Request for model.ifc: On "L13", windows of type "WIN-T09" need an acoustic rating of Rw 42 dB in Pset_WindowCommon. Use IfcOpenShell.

First a look at what the model holds.

```python
import ifcopenshell
import ifcopenshell.util.element

model = ifcopenshell.open("model.ifc")
print(model.schema)
storey = next(s for s in model.by_type("IfcBuildingStorey") if s.Name == "L13")
windows = [e for e in ifcopenshell.util.element.get_decomposition(storey) if e.is_a("IfcWindow")]
seen = {}
for e in windows:
    element_type = ifcopenshell.util.element.get_type(e)
    key = (element_type.Name if element_type != e and element_type else None, ifcopenshell.util.element.get_pset(e, "Pset_WindowCommon", "AcousticRating"))
    seen[key] = seen.get(key, 0) + 1
for (name, value), count in sorted(seen.items(), key=str):
    print(count, "x", name, "|", value)
```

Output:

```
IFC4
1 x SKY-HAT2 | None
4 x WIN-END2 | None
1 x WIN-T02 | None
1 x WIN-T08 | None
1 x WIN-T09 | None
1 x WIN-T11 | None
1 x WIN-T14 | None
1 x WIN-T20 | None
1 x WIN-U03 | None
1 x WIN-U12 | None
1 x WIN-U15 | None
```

```python
import ifcopenshell
import ifcopenshell.api.pset
import ifcopenshell.util.element

model = ifcopenshell.open("model.ifc")

storey = next(s for s in model.by_type("IfcBuildingStorey") if s.Name == "L13")
windows = [e for e in ifcopenshell.util.element.get_decomposition(storey) if e.is_a("IfcWindow")]

count = 0
for e in windows:
    element_type = ifcopenshell.util.element.get_type(e)
    if element_type in (None, e) or element_type.Name != "WIN-T09":
        continue
    # add_pset returns the element's existing set when there is one.
    pset = ifcopenshell.api.pset.add_pset(model, product=e, name="Pset_WindowCommon")
    ifcopenshell.api.pset.edit_pset(model, pset=pset, properties={"AcousticRating": "Rw 42 dB"})
    count += 1

print(count, "windows updated")

model.write("model_updated.ifc")
```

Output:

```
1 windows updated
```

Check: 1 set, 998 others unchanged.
